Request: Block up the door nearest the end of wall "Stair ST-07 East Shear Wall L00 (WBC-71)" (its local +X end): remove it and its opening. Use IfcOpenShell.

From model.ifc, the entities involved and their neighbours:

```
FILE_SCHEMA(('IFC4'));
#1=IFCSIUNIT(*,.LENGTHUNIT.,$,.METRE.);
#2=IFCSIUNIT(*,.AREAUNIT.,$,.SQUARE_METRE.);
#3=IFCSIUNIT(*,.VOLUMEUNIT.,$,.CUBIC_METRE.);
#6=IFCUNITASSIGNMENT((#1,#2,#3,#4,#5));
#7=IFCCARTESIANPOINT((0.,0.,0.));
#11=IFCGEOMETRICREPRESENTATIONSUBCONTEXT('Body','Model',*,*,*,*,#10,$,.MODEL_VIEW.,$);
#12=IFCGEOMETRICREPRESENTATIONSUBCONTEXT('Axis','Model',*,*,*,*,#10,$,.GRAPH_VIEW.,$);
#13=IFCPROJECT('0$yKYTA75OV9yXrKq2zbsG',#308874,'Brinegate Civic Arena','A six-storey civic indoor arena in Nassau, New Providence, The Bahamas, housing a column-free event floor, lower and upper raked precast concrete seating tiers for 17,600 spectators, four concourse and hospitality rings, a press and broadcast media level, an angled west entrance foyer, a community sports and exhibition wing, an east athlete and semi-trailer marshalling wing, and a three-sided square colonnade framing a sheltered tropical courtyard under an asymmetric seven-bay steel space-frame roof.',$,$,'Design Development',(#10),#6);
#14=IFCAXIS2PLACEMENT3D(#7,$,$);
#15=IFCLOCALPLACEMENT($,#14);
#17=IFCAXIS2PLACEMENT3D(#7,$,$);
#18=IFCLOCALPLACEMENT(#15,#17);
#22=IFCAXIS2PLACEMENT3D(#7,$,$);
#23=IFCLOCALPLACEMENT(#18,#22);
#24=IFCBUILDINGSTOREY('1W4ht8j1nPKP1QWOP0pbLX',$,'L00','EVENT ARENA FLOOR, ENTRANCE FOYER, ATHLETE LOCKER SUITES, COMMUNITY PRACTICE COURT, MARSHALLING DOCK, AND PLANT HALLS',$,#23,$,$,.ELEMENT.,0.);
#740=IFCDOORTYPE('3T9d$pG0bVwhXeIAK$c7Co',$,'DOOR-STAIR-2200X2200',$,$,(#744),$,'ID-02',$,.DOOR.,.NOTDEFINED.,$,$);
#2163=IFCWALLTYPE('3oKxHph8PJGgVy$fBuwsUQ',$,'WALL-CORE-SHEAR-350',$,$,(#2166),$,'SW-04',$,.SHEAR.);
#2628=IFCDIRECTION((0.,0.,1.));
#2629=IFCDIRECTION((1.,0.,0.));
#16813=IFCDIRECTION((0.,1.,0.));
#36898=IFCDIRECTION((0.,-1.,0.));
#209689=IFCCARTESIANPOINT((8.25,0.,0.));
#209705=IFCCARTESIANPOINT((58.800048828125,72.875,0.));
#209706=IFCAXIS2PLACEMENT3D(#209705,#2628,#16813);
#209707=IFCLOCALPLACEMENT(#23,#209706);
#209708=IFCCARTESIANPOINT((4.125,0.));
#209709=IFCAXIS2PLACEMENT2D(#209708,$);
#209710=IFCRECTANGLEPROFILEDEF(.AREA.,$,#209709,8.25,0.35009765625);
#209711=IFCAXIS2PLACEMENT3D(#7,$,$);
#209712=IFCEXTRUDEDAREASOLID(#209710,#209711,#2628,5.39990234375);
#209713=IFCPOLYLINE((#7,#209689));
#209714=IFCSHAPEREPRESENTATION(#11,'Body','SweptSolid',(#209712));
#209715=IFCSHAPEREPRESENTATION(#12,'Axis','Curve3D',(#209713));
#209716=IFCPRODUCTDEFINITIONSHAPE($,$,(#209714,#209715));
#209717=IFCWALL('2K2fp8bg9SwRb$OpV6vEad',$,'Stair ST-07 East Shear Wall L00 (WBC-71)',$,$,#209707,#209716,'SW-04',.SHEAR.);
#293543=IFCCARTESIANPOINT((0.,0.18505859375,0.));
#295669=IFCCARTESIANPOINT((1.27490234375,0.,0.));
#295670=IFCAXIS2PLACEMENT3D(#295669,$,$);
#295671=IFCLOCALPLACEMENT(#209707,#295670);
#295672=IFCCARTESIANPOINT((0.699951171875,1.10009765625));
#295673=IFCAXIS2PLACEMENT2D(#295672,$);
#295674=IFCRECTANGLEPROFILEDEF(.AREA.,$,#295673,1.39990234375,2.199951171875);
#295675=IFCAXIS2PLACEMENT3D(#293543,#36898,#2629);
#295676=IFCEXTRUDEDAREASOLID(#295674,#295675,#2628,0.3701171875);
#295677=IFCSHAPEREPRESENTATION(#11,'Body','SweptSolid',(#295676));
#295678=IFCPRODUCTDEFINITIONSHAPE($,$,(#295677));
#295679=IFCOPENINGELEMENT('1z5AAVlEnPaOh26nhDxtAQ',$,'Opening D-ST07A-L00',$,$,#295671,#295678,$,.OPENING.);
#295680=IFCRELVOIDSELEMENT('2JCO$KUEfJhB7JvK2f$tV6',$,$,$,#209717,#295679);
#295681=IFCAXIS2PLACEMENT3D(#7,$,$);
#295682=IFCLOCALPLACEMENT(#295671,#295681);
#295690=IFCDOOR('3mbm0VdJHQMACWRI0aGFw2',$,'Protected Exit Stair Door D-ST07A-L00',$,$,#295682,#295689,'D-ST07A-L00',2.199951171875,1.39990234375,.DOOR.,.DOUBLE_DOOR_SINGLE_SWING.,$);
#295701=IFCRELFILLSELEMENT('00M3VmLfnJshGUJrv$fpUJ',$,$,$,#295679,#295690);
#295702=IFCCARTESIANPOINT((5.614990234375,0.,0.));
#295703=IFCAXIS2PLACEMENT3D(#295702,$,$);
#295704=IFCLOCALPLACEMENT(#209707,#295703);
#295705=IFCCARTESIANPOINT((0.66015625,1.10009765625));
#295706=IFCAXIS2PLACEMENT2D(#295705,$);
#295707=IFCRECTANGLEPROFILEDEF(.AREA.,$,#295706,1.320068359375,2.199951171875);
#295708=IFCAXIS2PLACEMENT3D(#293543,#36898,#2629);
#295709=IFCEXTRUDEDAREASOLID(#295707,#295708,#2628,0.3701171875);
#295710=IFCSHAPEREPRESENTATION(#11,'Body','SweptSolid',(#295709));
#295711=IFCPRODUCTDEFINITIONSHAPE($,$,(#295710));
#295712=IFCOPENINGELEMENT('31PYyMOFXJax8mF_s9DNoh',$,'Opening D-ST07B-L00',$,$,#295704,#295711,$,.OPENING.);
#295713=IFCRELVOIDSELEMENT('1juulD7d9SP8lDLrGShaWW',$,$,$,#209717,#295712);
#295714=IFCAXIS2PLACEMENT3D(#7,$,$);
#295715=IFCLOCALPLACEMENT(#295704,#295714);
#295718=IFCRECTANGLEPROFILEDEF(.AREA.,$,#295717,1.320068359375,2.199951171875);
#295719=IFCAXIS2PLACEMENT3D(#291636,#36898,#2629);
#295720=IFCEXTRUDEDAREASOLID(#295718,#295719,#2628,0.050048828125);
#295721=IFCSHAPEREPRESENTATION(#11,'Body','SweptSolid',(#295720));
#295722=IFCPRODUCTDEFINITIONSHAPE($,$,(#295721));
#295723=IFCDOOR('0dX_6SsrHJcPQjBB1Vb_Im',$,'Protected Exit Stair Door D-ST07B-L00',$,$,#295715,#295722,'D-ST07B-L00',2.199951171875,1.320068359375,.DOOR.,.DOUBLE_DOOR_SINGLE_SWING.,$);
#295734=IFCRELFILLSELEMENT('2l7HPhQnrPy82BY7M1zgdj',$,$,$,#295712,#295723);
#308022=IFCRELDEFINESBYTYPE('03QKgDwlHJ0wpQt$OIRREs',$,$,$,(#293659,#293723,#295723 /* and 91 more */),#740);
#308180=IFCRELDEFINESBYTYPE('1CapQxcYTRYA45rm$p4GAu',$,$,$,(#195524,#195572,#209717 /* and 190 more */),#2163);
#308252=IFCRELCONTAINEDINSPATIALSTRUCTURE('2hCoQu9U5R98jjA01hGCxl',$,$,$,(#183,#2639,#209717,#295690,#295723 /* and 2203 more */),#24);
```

```python
import ifcopenshell
import ifcopenshell.api.feature
import ifcopenshell.api.root
import ifcopenshell.geom
import ifcopenshell.util.shape

model = ifcopenshell.open("model.ifc")
settings = ifcopenshell.geom.settings()


def volume(element):
    """Net volume in cubic metres, openings subtracted."""
    shape = ifcopenshell.geom.create_shape(settings, element)
    return ifcopenshell.util.shape.get_volume(shape.geometry)


door = model.by_id(295723)
opening = door.FillsVoids[0].RelatingOpeningElement
wall = opening.VoidsElements[0].RelatingBuildingElement
before = volume(wall)

ifcopenshell.api.root.remove_product(model, product=door)
ifcopenshell.api.feature.remove_feature(model, feature=opening)

after = volume(wall)

print(f"wall volume {before:.3f} -> {after:.3f} m3")

model.write("model_v2.ifc")
```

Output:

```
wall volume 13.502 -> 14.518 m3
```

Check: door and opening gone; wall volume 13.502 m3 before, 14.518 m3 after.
